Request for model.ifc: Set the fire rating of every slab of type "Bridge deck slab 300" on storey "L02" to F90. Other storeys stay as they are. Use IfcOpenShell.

First a look at what the model holds.

```python
import ifcopenshell
import ifcopenshell.util.element

model = ifcopenshell.open("model.ifc")
print(model.schema)
storey = next(s for s in model.by_type("IfcBuildingStorey") if s.Name == "L02")
slabs = [e for e in ifcopenshell.util.element.get_decomposition(storey) if e.is_a("IfcSlab")]
seen = {}
for e in slabs:
    element_type = ifcopenshell.util.element.get_type(e)
    key = (element_type.Name if element_type != e and element_type else None, ifcopenshell.util.element.get_pset(e, "Pset_SlabCommon", "FireRating"))
    seen[key] = seen.get(key, 0) + 1
for (name, value), count in sorted(seen.items(), key=str):
    print(count, "x", name, "|", value)
```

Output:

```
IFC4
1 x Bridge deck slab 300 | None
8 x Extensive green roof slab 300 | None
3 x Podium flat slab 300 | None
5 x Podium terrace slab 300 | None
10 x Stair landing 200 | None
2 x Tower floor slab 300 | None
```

```python
import ifcopenshell
import ifcopenshell.api.pset
import ifcopenshell.util.element

model = ifcopenshell.open("model.ifc")

storey = next(s for s in model.by_type("IfcBuildingStorey") if s.Name == "L02")
slabs = [e for e in ifcopenshell.util.element.get_decomposition(storey) if e.is_a("IfcSlab")]

count = 0
for e in slabs:
    element_type = ifcopenshell.util.element.get_type(e)
    if element_type in (None, e) or element_type.Name != "Bridge deck slab 300":
        continue
    found = ifcopenshell.util.element.get_pset(e, "Pset_SlabCommon", should_inherit=False)
    if found:
        pset = model.by_id(found["id"])
        if len(ifcopenshell.util.element.get_elements_by_pset(pset)) > 1:
            pset = ifcopenshell.api.pset.unshare_pset(model, products=[e], pset=pset)[0]
    else:
        pset = ifcopenshell.api.pset.add_pset(model, product=e, name="Pset_SlabCommon")
    ifcopenshell.api.pset.edit_pset(model, pset=pset, properties={"FireRating": "F90"})
    count += 1

print(count, "slabs updated")

model.write("model_rev.ifc")
```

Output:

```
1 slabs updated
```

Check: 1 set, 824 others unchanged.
